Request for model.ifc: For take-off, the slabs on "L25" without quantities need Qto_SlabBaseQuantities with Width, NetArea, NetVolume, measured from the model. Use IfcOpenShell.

First a look at what the model holds.

```python
import ifcopenshell
import ifcopenshell.util.element
import ifcopenshell.util.unit

model = ifcopenshell.open("model.ifc")
print(model.schema)
for unit_type in ("LENGTHUNIT", "AREAUNIT", "VOLUMEUNIT"):
    print(unit_type, ifcopenshell.util.unit.calculate_unit_scale(model, unit_type))
storey = next(s for s in model.by_type("IfcBuildingStorey") if s.Name == "L25")
slabs = [e for e in ifcopenshell.util.element.get_decomposition(storey) if e.is_a("IfcSlab")]
for e in sorted(slabs, key=lambda e: e.id()):
    print(e.id(), e.is_a(), e.Name, list(ifcopenshell.util.element.get_psets(e, qtos_only=True)), sep=" | ")
```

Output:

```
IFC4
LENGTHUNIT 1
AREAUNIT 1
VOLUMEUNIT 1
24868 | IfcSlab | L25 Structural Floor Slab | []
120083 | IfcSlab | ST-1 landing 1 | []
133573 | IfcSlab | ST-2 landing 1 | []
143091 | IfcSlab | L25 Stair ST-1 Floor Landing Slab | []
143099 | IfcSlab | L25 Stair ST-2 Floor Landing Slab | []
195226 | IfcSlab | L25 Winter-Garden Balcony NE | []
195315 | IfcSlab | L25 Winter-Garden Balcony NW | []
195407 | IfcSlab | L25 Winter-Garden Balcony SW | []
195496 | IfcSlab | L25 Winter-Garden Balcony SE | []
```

```python
import ifcopenshell
import ifcopenshell.api.pset
import ifcopenshell.geom
import ifcopenshell.util.element
import ifcopenshell.util.shape
import ifcopenshell.util.unit

model = ifcopenshell.open("model.ifc")
unit_scale = ifcopenshell.util.unit.calculate_unit_scale(model)
area_scale = ifcopenshell.util.unit.calculate_unit_scale(model, "AREAUNIT")
volume_scale = ifcopenshell.util.unit.calculate_unit_scale(model, "VOLUMEUNIT")
settings = ifcopenshell.geom.settings()

storey = next(s for s in model.by_type("IfcBuildingStorey") if s.Name == "L25")
slabs = [e for e in ifcopenshell.util.element.get_decomposition(storey) if e.is_a("IfcSlab")]

for e in sorted(slabs, key=lambda e: e.id()):
    if ifcopenshell.util.element.get_psets(e, qtos_only=True, should_inherit=False):
        continue
    # Geometry comes back in metres, in the element's own axes.
    shape = ifcopenshell.geom.create_shape(settings, e)
    values = {
        "Width": ifcopenshell.util.shape.get_z(shape.geometry) / unit_scale,
        "NetArea": ifcopenshell.util.shape.get_footprint_area(shape.geometry) / area_scale,
        "NetVolume": ifcopenshell.util.shape.get_volume(shape.geometry) / volume_scale,
    }
    qto = ifcopenshell.api.pset.add_qto(model, product=e, name="Qto_SlabBaseQuantities")
    ifcopenshell.api.pset.edit_qto(model, qto=qto, properties=values)
    print(e.id(), {k: round(v, 3) for k, v in values.items()})

model.write("model_rev.ifc")
```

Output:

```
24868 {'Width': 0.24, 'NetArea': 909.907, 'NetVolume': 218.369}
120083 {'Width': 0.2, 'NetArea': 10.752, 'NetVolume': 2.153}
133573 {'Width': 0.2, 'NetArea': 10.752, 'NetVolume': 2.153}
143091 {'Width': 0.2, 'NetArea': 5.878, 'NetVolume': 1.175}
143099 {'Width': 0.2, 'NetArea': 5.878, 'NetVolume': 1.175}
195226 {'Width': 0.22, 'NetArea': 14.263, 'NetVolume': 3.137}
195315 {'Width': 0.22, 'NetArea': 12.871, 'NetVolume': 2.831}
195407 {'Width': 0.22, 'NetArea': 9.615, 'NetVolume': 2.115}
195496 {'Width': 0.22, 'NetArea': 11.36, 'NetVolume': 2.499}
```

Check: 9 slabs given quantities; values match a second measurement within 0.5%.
